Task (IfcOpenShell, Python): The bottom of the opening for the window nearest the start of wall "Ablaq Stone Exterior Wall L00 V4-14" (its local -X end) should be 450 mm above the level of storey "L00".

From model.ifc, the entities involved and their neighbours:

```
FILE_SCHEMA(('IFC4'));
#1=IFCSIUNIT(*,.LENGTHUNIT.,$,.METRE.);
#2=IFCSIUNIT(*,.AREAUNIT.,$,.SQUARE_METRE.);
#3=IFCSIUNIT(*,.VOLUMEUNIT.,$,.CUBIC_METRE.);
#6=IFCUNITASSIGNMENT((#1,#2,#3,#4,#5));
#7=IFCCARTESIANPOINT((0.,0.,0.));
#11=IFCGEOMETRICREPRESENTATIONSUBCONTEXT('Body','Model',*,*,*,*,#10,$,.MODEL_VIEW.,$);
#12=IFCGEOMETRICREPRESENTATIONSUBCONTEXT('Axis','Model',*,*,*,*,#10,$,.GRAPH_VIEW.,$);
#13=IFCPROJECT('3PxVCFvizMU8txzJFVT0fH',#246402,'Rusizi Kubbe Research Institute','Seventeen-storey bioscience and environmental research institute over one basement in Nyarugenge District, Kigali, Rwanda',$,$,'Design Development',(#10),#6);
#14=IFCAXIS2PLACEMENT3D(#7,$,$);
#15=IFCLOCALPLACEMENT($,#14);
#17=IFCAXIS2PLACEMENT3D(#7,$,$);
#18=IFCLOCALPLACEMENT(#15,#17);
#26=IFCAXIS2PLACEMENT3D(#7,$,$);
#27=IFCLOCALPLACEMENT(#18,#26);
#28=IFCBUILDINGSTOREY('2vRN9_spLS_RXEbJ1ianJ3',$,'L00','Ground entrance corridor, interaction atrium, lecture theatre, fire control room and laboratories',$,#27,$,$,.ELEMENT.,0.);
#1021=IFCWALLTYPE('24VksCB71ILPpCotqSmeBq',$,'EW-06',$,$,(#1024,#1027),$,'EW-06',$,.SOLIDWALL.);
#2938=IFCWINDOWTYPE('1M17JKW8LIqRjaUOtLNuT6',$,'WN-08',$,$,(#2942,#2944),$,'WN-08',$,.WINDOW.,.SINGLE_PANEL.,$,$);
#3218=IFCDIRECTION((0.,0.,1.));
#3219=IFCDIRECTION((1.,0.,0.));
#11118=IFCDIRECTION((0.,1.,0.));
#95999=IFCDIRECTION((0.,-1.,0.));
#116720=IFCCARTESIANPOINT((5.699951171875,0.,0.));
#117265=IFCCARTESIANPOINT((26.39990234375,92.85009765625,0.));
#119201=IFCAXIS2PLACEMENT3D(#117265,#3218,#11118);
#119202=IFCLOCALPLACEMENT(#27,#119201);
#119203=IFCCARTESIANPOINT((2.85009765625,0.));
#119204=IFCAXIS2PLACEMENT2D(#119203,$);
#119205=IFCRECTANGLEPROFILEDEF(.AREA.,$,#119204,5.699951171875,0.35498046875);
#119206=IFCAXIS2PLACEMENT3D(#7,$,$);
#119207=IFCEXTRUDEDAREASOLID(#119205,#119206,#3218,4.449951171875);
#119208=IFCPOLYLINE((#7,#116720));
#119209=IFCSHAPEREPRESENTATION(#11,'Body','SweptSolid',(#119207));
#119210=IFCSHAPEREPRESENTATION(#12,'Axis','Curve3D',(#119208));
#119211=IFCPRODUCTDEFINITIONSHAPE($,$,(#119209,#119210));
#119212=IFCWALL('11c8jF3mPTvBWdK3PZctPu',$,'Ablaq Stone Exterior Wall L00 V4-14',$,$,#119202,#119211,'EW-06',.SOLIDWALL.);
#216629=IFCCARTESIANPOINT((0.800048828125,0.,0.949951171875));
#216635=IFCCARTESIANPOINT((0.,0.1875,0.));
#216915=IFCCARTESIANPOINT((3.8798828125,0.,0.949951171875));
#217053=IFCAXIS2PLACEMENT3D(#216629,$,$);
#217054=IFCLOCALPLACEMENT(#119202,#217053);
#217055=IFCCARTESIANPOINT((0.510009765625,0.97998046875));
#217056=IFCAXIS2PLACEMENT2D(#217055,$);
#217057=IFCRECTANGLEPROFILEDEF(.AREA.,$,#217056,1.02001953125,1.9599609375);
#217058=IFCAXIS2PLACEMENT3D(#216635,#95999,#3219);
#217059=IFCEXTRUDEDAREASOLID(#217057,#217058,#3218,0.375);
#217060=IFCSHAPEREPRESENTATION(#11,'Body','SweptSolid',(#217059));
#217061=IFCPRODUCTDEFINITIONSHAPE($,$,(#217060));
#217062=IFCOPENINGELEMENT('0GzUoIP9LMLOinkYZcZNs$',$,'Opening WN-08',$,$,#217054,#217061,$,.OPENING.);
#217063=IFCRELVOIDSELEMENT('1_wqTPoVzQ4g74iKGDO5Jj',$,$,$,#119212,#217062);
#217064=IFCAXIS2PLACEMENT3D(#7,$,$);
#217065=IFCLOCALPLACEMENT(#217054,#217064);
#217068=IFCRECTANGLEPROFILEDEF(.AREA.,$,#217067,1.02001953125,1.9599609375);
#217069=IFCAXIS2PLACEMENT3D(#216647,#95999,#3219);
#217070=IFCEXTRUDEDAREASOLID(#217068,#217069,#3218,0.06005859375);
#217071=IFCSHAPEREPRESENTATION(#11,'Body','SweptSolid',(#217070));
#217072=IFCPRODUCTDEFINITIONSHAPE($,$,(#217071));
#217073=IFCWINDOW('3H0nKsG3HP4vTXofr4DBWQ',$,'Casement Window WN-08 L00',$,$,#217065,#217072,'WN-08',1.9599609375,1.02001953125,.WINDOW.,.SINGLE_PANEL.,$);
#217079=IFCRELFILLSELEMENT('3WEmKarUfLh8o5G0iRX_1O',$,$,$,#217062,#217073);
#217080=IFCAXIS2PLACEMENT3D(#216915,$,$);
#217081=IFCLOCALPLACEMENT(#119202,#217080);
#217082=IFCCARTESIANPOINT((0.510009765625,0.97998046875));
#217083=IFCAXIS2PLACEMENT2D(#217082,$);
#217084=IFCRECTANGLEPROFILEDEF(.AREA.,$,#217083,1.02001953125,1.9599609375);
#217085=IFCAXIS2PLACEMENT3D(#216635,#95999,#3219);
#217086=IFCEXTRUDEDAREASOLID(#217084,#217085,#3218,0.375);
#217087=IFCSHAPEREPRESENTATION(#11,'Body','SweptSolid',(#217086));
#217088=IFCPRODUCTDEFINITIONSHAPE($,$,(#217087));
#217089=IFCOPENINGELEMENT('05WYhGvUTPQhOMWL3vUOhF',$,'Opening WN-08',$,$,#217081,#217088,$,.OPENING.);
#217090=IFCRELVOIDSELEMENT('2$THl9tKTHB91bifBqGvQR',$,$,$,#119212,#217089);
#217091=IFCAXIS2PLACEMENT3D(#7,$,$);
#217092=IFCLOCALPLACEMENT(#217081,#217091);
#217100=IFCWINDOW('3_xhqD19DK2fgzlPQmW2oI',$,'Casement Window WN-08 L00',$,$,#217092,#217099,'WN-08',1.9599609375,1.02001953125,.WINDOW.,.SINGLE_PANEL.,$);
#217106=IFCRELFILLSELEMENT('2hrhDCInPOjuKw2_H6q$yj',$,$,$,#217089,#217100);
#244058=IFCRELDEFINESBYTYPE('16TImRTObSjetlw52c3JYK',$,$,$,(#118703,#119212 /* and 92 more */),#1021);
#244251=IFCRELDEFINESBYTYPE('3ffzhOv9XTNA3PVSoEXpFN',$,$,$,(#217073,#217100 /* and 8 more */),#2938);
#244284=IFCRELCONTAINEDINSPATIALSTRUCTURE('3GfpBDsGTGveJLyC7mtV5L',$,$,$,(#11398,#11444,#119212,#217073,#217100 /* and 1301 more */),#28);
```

```python
import numpy as np
import ifcopenshell
import ifcopenshell.api.geometry
import ifcopenshell.geom
import ifcopenshell.util.element
import ifcopenshell.util.placement
import ifcopenshell.util.shape
import ifcopenshell.util.unit

model = ifcopenshell.open("model.ifc")
unit_scale = ifcopenshell.util.unit.calculate_unit_scale(model)

window = model.by_id(217073)
opening = window.FillsVoids[0].RelatingOpeningElement
storey = ifcopenshell.util.element.get_container(window, ifc_class="IfcBuildingStorey")
level = ifcopenshell.util.placement.get_local_placement(storey.ObjectPlacement)[2, 3]

# The opening's origin need not be at the sill, so measure its lowest point.
shape = ifcopenshell.geom.create_shape(ifcopenshell.geom.settings(), opening)
bottom = ifcopenshell.util.shape.get_shape_bottom_elevation(shape, shape.geometry) / unit_scale
dz = level + 0.45 - bottom

shift = np.array([0.0, 0.0, dz])
# The window is placed relative to its opening, so it follows when the opening moves.
matrix = ifcopenshell.util.placement.get_local_placement(opening.ObjectPlacement)
matrix[:3, 3] += shift
ifcopenshell.api.geometry.edit_object_placement(
    model, product=opening, matrix=matrix, is_si=False, should_transform_children=True
)

print(f"moved by {dz * unit_scale:+.3f} m")

model.write("model_rev.ifc")
```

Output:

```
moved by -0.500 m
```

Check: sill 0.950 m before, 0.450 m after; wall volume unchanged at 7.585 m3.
